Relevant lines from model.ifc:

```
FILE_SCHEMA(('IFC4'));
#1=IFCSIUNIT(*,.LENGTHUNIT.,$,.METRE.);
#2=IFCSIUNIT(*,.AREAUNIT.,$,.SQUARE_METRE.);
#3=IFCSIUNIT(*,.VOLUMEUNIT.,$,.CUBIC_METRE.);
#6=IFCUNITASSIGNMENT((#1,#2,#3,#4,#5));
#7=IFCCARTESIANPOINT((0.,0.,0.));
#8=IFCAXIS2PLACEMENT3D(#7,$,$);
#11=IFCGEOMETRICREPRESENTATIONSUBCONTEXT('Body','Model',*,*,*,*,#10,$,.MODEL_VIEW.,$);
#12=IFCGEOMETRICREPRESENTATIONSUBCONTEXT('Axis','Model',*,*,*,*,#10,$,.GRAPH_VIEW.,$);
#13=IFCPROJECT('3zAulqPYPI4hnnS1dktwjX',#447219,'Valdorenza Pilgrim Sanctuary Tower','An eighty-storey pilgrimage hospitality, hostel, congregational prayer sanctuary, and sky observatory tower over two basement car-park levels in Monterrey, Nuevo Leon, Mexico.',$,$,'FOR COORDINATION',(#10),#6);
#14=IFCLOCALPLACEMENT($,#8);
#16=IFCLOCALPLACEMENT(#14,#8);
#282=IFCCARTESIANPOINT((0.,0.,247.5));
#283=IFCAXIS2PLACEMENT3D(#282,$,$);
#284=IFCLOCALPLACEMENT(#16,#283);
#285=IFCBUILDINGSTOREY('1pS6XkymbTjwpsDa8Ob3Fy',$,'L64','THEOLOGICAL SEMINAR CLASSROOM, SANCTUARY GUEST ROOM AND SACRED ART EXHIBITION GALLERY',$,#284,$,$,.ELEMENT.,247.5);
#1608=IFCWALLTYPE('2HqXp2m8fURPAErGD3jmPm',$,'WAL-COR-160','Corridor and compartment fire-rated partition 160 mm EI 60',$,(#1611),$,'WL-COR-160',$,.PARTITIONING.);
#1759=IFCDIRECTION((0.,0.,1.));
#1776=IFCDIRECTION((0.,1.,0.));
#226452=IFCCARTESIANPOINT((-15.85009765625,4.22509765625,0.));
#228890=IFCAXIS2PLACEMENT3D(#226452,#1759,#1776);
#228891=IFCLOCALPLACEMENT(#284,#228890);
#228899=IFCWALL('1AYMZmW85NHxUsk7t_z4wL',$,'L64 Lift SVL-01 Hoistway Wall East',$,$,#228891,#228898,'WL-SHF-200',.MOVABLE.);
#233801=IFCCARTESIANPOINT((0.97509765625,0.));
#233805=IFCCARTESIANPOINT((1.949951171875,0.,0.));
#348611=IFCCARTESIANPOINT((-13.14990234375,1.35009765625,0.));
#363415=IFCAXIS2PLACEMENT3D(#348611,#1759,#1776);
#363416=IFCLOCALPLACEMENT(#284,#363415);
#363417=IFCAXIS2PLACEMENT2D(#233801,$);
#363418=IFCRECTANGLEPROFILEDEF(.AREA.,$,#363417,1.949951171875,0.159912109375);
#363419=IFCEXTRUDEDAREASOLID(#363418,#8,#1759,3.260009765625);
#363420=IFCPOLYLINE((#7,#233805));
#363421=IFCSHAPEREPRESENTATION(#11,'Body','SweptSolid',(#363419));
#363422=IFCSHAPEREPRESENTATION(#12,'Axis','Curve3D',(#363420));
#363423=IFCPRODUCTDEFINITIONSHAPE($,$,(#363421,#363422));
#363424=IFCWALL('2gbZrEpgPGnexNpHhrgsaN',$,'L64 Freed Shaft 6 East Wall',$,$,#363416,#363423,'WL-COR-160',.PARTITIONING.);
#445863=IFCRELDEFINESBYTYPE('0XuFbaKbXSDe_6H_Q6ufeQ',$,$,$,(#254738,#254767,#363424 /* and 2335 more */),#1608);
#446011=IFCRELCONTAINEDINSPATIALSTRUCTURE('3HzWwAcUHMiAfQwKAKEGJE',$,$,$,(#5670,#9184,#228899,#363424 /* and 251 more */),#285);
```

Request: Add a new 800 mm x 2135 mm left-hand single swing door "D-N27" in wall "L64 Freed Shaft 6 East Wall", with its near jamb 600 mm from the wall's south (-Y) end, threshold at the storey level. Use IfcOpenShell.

```python
import numpy as np
import ifcopenshell
import ifcopenshell.api.feature
import ifcopenshell.api.geometry
import ifcopenshell.api.root
import ifcopenshell.api.spatial
import ifcopenshell.geom
import ifcopenshell.util.element
import ifcopenshell.util.placement
import ifcopenshell.util.representation
import ifcopenshell.util.shape
import ifcopenshell.util.unit

model = ifcopenshell.open("model.ifc")
unit_scale = ifcopenshell.util.unit.calculate_unit_scale(model)
settings = ifcopenshell.geom.settings()


def volume(element):
    """Net volume in cubic metres, openings subtracted."""
    shape = ifcopenshell.geom.create_shape(settings, element)
    return ifcopenshell.util.shape.get_volume(shape.geometry)


wall = model.by_id(363424)
storey = ifcopenshell.util.element.get_container(wall, ifc_class="IfcBuildingStorey")
context = ifcopenshell.util.representation.get_context(model, "Model", "Body", "MODEL_VIEW")
before = volume(wall)

width, height, from_end, sill = 0.8, 2.135, 0.6, 0.0  # metres

# The wall runs along its own X axis, and the end named is its -X end.
wall_shape = ifcopenshell.geom.create_shape(settings, wall)
x, y, z = ifcopenshell.util.shape.get_vertices(wall_shape.geometry).T
start = x.min() + from_end
face, thickness = float(y.min()), float(y.max() - y.min())
wall_matrix = ifcopenshell.util.placement.get_local_placement(wall.ObjectPlacement)
level = ifcopenshell.util.placement.get_local_placement(storey.ObjectPlacement)[2, 3]


def in_wall(x, y):
    """Placement at x, y metres in the wall's axes, at sill height."""
    matrix = wall_matrix.copy()
    matrix[:, 3] = wall_matrix @ np.array([x / unit_scale, y / unit_scale, 0.0, 1.0])
    matrix[2, 3] = level + sill / unit_scale
    return matrix


# Opening: a box that overshoots both wall faces by 50 mm.
opening = ifcopenshell.api.root.create_entity(model, ifc_class="IfcOpeningElement", predefined_type="OPENING")
box = ifcopenshell.api.geometry.add_wall_representation(
    model, context=context, length=width, height=height, thickness=thickness + 0.1
)
ifcopenshell.api.geometry.assign_representation(model, product=opening, representation=box)
ifcopenshell.api.geometry.edit_object_placement(model, product=opening, matrix=in_wall(start, face - 0.05), is_si=False)
ifcopenshell.api.feature.add_feature(model, feature=opening, element=wall)

door = ifcopenshell.api.root.create_entity(model, ifc_class="IfcDoor", name="D-N27", predefined_type="DOOR")
door.OverallWidth, door.OverallHeight = width / unit_scale, height / unit_scale
door.OperationType = "SINGLE_SWING_LEFT"
body = ifcopenshell.api.geometry.add_door_representation(
    model,
    context=context,
    overall_width=door.OverallWidth,
    overall_height=door.OverallHeight,
    operation_type="SINGLE_SWING_LEFT",
    lining_properties={"LiningDepth": thickness / unit_scale, "ThresholdDepth": thickness / unit_scale},
)
ifcopenshell.api.geometry.assign_representation(model, product=door, representation=body)
ifcopenshell.api.spatial.assign_container(model, products=[door], relating_structure=storey)
ifcopenshell.api.feature.add_filling(model, opening=opening, element=door)

# The lining spans the wall, so the door starts at the wall face.
ifcopenshell.api.geometry.edit_object_placement(model, product=door, matrix=in_wall(start, face), is_si=False)

after = volume(wall)

print(f"wall volume {before:.3f} -> {after:.3f} m3")

model.write("model-out.ifc")
```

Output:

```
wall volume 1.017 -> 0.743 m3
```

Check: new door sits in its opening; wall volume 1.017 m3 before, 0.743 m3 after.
